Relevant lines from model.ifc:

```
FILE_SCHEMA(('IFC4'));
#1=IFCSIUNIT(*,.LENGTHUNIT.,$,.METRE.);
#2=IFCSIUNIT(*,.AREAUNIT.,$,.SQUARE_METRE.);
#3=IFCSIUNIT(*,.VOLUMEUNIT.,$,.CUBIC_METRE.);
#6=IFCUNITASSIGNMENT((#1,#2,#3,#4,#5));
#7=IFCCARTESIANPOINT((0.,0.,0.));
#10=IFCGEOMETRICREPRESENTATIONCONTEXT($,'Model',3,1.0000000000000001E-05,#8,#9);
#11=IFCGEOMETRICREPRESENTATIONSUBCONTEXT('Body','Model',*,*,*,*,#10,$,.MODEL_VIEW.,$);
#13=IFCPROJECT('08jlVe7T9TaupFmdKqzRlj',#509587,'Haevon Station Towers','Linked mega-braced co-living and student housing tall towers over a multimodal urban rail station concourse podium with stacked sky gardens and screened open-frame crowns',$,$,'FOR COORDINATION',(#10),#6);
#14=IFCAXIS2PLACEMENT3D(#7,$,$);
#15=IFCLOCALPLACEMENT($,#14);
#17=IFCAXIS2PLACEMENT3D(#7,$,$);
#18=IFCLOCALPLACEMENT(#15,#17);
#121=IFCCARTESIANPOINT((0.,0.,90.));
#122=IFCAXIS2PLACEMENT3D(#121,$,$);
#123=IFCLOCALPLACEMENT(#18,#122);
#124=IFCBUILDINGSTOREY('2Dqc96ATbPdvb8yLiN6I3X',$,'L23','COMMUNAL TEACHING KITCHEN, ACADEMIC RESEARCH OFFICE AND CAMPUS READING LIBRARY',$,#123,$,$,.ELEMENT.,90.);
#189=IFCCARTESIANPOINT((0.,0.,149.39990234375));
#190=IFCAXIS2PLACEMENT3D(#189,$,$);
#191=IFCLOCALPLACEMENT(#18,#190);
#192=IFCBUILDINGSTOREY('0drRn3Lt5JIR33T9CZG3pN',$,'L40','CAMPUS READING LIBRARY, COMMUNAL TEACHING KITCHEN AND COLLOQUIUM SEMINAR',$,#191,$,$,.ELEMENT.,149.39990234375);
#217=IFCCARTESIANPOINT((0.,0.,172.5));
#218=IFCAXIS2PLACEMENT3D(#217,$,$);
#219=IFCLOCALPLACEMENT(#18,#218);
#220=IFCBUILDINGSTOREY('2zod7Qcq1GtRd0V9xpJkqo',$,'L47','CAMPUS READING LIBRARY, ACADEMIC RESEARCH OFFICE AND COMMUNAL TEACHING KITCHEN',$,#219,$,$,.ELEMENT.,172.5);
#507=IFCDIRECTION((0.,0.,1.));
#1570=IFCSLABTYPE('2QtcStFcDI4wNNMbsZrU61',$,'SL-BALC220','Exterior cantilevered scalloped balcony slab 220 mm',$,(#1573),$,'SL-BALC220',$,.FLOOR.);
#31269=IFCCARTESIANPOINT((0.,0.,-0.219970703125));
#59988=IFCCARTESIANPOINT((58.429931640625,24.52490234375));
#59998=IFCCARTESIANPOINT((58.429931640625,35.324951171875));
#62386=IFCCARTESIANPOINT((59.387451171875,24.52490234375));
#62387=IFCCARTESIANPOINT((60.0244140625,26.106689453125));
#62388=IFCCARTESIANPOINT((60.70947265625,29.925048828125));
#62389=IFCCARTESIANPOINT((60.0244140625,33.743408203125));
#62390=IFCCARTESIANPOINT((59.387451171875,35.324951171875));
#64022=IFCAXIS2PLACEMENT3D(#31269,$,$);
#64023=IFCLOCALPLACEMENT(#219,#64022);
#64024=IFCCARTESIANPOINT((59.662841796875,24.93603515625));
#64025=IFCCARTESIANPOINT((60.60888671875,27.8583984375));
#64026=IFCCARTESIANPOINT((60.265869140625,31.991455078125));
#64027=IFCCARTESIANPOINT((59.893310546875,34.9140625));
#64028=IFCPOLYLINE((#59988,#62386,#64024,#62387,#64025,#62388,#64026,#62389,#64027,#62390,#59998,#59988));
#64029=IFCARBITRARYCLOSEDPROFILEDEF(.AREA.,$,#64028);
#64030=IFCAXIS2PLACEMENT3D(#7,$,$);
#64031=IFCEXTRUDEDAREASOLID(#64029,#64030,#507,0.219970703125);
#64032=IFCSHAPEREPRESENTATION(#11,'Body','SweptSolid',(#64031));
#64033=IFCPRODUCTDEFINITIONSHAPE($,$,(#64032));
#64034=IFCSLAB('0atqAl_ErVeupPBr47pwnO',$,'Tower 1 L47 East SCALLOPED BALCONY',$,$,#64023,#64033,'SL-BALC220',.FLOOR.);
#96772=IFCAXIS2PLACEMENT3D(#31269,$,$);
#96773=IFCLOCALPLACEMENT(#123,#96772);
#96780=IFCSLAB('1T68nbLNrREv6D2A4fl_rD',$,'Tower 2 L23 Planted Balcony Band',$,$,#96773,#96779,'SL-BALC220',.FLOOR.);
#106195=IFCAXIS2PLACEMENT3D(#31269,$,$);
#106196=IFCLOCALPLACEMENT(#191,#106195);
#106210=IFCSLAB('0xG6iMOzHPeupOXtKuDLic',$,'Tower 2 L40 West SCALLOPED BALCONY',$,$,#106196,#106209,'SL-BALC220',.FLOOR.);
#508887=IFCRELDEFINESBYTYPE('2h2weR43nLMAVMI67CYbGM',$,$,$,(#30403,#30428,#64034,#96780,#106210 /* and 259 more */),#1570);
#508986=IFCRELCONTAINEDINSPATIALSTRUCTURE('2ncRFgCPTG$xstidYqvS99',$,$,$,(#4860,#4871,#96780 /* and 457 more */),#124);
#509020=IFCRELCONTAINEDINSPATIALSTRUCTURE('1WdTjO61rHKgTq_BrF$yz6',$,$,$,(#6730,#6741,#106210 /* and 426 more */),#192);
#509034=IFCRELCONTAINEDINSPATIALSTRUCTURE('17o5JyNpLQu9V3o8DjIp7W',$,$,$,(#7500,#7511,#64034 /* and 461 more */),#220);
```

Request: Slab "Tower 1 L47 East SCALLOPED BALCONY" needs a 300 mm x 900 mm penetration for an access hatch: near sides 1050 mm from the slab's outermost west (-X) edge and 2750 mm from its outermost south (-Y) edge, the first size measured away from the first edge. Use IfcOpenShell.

```python
import numpy as np
import ifcopenshell
import ifcopenshell.api.feature
import ifcopenshell.api.geometry
import ifcopenshell.api.root
import ifcopenshell.geom
import ifcopenshell.util.placement
import ifcopenshell.util.representation
import ifcopenshell.util.shape
import ifcopenshell.util.unit

model = ifcopenshell.open("model.ifc")
unit_scale = ifcopenshell.util.unit.calculate_unit_scale(model)
settings = ifcopenshell.geom.settings()


def volume(element):
    """Net volume in cubic metres, openings subtracted."""
    shape = ifcopenshell.geom.create_shape(settings, element)
    return ifcopenshell.util.shape.get_volume(shape.geometry)


slab = model.by_guid("0atqAl_ErVeupPBr47pwnO")
before = volume(slab)

# Extent in the slab's own axes, in metres. The edges named are its -X and -Y sides.
slab_shape = ifcopenshell.geom.create_shape(settings, slab)
vertices = ifcopenshell.util.shape.get_vertices(slab_shape.geometry)
x_min, y_min, bottom = vertices.min(axis=0)
top = vertices[:, 2].max()

opening = ifcopenshell.api.root.create_entity(model, ifc_class="IfcOpeningElement", name="Access hatch opening", predefined_type="OPENING")
context = ifcopenshell.util.representation.get_context(model, "Model", "Body", "MODEL_VIEW")
width, depth = 0.3, 0.9
outline = [(0.0, 0.0), (width, 0.0), (width, depth), (0.0, depth), (0.0, 0.0)]
# Overshoot both faces by 50 mm so the cut is clean.
shape = ifcopenshell.api.geometry.add_slab_representation(
    model, context=context, depth=top - bottom + 0.1, polyline=outline
)
ifcopenshell.api.geometry.assign_representation(model, product=opening, representation=shape)

matrix = ifcopenshell.util.placement.get_local_placement(slab.ObjectPlacement)
matrix[:, 3] = matrix @ np.append(np.array([x_min + 1.05, y_min + 2.75, bottom - 0.05]) / unit_scale, 1.0)
ifcopenshell.api.geometry.edit_object_placement(model, product=opening, matrix=matrix, is_si=False)
ifcopenshell.api.feature.add_feature(model, feature=opening, element=slab)

after = volume(slab)

print(f"slab volume {before:.3f} -> {after:.3f} m3")

model.write("model_v2.ifc")
```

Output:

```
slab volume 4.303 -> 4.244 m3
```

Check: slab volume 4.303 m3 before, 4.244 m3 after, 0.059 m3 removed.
